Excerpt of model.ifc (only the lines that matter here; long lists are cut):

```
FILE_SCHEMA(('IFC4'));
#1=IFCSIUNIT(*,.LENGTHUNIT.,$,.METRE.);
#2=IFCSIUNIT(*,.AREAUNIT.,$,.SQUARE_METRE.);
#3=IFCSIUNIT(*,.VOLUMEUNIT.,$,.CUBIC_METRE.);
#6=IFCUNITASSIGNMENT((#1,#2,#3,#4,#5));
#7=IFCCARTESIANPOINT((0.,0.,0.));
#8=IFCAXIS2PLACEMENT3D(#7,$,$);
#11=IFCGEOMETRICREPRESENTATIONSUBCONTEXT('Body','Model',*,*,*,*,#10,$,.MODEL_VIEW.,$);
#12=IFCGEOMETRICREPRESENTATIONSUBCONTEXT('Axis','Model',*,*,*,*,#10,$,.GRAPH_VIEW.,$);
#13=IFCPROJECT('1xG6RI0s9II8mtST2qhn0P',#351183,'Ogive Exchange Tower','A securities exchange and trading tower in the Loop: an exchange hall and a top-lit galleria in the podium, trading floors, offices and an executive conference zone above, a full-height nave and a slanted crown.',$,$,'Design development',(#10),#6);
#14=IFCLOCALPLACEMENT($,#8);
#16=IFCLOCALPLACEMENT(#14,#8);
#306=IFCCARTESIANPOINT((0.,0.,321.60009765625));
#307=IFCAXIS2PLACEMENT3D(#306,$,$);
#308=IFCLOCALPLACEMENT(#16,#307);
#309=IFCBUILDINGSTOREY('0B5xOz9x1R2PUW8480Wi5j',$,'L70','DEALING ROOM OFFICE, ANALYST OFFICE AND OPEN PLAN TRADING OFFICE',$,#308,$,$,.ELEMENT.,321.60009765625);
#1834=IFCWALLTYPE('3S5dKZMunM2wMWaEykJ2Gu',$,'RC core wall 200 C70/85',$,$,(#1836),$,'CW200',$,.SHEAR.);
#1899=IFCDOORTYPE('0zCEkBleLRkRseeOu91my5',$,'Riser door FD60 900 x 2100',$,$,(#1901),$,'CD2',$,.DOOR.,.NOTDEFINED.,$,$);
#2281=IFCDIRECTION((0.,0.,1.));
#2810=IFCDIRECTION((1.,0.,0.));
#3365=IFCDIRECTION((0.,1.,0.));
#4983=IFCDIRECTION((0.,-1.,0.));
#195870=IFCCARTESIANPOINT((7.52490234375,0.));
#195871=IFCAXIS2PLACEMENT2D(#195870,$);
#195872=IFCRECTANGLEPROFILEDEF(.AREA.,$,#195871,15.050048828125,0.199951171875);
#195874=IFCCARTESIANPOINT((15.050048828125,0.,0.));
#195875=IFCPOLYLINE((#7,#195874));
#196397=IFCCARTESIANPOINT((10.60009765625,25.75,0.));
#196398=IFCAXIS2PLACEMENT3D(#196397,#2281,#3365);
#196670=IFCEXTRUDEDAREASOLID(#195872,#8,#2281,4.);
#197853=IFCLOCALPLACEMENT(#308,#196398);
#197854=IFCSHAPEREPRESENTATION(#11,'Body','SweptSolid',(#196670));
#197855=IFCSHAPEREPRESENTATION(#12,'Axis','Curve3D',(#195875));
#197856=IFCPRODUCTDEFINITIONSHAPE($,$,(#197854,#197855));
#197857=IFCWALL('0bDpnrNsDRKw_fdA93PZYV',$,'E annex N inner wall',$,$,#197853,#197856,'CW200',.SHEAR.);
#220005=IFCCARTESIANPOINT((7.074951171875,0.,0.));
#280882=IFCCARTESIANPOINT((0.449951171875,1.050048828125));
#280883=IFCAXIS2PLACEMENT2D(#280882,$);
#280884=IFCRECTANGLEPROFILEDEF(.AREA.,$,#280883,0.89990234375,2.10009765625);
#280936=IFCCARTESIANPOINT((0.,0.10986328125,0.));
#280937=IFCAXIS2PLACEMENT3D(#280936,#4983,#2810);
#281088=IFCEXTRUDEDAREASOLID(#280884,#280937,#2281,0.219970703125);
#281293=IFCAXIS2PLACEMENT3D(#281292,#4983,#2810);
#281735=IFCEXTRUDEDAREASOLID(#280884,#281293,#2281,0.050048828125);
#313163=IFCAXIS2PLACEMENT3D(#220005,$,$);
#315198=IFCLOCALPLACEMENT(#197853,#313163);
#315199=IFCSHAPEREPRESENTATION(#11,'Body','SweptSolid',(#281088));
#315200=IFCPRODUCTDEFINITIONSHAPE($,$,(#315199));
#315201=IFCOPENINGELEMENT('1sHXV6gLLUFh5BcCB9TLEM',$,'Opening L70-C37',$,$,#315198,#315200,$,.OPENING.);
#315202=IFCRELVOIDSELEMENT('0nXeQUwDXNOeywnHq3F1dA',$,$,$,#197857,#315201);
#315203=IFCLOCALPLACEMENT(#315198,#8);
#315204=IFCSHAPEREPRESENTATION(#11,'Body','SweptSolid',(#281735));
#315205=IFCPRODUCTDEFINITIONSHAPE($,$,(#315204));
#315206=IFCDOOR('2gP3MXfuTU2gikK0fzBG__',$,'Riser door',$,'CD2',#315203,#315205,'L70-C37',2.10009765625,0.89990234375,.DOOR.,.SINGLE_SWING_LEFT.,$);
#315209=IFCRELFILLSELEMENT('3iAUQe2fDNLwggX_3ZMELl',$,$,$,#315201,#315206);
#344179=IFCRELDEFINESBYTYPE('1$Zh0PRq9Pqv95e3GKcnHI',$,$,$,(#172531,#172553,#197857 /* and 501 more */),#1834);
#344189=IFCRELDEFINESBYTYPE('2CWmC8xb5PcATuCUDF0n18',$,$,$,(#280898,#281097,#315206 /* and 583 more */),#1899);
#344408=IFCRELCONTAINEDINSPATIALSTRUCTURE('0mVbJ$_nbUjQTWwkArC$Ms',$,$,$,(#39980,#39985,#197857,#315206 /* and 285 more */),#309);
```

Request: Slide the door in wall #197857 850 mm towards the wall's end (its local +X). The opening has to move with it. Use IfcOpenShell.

```python
import ifcopenshell
import ifcopenshell.api.geometry
import ifcopenshell.util.placement

model = ifcopenshell.open("model.ifc")

door = model.by_id(315206)
opening = door.FillsVoids[0].RelatingOpeningElement
wall = opening.VoidsElements[0].RelatingBuildingElement

wall_matrix = ifcopenshell.util.placement.get_local_placement(wall.ObjectPlacement)
shift = wall_matrix[:3, 0] * 0.85
before = ifcopenshell.util.placement.get_local_placement(door.ObjectPlacement)[:3, 3].copy()

# The door is placed relative to its opening, so it follows when the opening moves.
matrix = ifcopenshell.util.placement.get_local_placement(opening.ObjectPlacement)
matrix[:3, 3] += shift
ifcopenshell.api.geometry.edit_object_placement(
    model, product=opening, matrix=matrix, is_si=False, should_transform_children=True
)

after = ifcopenshell.util.placement.get_local_placement(door.ObjectPlacement)[:3, 3]
print("door moved by", (after - before).round(3) + 0.0)

model.write("model-out.ifc")
```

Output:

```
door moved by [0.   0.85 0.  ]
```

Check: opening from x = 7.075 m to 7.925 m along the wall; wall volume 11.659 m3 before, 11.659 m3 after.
